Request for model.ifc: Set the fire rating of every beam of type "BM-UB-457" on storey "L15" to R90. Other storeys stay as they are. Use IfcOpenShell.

First a look at what the model holds.

```python
import ifcopenshell
import ifcopenshell.util.element

model = ifcopenshell.open("model.ifc")
print(model.schema)
storey = next(s for s in model.by_type("IfcBuildingStorey") if s.Name == "L15")
beams = [e for e in ifcopenshell.util.element.get_decomposition(storey) if e.is_a("IfcBeam")]
seen = {}
for e in beams:
    element_type = ifcopenshell.util.element.get_type(e)
    key = (element_type.Name if element_type != e and element_type else None, ifcopenshell.util.element.get_pset(e, "Pset_BeamCommon", "FireRating"))
    seen[key] = seen.get(key, 0) + 1
for (name, value), count in sorted(seen.items(), key=str):
    print(count, "x", name, "|", value)
```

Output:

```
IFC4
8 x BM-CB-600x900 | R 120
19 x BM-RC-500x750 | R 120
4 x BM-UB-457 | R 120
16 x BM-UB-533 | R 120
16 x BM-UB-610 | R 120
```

```python
import ifcopenshell
import ifcopenshell.api.pset
import ifcopenshell.util.element

model = ifcopenshell.open("model.ifc")

storey = next(s for s in model.by_type("IfcBuildingStorey") if s.Name == "L15")
beams = [e for e in ifcopenshell.util.element.get_decomposition(storey) if e.is_a("IfcBeam")]

count = 0
for e in beams:
    element_type = ifcopenshell.util.element.get_type(e)
    if element_type in (None, e) or element_type.Name != "BM-UB-457":
        continue
    # add_pset returns the element's existing set when there is one.
    pset = ifcopenshell.api.pset.add_pset(model, product=e, name="Pset_BeamCommon")
    ifcopenshell.api.pset.edit_pset(model, pset=pset, properties={"FireRating": "R90"})
    count += 1

print(count, "beams updated")

model.write("model_updated.ifc")
```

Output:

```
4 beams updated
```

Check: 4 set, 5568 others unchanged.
